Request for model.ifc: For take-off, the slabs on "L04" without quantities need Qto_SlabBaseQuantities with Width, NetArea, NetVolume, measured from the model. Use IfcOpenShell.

First a look at what the model holds.

```python
import ifcopenshell
import ifcopenshell.util.element
import ifcopenshell.util.unit

model = ifcopenshell.open("model.ifc")
print(model.schema)
for unit_type in ("LENGTHUNIT", "AREAUNIT", "VOLUMEUNIT"):
    print(unit_type, ifcopenshell.util.unit.calculate_unit_scale(model, unit_type))
storey = next(s for s in model.by_type("IfcBuildingStorey") if s.Name == "L04")
slabs = [e for e in ifcopenshell.util.element.get_decomposition(storey) if e.is_a("IfcSlab")]
for e in sorted(slabs, key=lambda e: e.id()):
    print(e.id(), e.is_a(), e.Name, list(ifcopenshell.util.element.get_psets(e, qtos_only=True)), sep=" | ")
```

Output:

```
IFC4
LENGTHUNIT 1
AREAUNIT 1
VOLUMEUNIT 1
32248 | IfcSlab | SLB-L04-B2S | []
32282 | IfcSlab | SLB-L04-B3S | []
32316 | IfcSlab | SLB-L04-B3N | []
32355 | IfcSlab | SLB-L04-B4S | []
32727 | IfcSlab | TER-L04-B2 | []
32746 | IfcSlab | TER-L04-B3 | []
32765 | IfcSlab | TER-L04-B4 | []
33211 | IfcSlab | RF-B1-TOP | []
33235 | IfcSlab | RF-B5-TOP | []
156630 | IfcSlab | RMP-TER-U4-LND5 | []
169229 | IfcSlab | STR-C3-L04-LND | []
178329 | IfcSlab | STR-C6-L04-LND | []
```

```python
import ifcopenshell
import ifcopenshell.api.pset
import ifcopenshell.geom
import ifcopenshell.util.element
import ifcopenshell.util.shape
import ifcopenshell.util.unit

model = ifcopenshell.open("model.ifc")
unit_scale = ifcopenshell.util.unit.calculate_unit_scale(model)
area_scale = ifcopenshell.util.unit.calculate_unit_scale(model, "AREAUNIT")
volume_scale = ifcopenshell.util.unit.calculate_unit_scale(model, "VOLUMEUNIT")
settings = ifcopenshell.geom.settings()

storey = next(s for s in model.by_type("IfcBuildingStorey") if s.Name == "L04")
slabs = [e for e in ifcopenshell.util.element.get_decomposition(storey) if e.is_a("IfcSlab")]

for e in sorted(slabs, key=lambda e: e.id()):
    if ifcopenshell.util.element.get_psets(e, qtos_only=True, should_inherit=False):
        continue
    # Geometry comes back in metres, in the element's own axes.
    shape = ifcopenshell.geom.create_shape(settings, e)
    values = {
        "Width": ifcopenshell.util.shape.get_z(shape.geometry) / unit_scale,
        "NetArea": ifcopenshell.util.shape.get_footprint_area(shape.geometry) / area_scale,
        "NetVolume": ifcopenshell.util.shape.get_volume(shape.geometry) / volume_scale,
    }
    qto = ifcopenshell.api.pset.add_qto(model, product=e, name="Qto_SlabBaseQuantities")
    ifcopenshell.api.pset.edit_qto(model, qto=qto, properties=values)
    print(e.id(), {k: round(v, 3) for k, v in values.items()})

model.write("model_rev.ifc")
```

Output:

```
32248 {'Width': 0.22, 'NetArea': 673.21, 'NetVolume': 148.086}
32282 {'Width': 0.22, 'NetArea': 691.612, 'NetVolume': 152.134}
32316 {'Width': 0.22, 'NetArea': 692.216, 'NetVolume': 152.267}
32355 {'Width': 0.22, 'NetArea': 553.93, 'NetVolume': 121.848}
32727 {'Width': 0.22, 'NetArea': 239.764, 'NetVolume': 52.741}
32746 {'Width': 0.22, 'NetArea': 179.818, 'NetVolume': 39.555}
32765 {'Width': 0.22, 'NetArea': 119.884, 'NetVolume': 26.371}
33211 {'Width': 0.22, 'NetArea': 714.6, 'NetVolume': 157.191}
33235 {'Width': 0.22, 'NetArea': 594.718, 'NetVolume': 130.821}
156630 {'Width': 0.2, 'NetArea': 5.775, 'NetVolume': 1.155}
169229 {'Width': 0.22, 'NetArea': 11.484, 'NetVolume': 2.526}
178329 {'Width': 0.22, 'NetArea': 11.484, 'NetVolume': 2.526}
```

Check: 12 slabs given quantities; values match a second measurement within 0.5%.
